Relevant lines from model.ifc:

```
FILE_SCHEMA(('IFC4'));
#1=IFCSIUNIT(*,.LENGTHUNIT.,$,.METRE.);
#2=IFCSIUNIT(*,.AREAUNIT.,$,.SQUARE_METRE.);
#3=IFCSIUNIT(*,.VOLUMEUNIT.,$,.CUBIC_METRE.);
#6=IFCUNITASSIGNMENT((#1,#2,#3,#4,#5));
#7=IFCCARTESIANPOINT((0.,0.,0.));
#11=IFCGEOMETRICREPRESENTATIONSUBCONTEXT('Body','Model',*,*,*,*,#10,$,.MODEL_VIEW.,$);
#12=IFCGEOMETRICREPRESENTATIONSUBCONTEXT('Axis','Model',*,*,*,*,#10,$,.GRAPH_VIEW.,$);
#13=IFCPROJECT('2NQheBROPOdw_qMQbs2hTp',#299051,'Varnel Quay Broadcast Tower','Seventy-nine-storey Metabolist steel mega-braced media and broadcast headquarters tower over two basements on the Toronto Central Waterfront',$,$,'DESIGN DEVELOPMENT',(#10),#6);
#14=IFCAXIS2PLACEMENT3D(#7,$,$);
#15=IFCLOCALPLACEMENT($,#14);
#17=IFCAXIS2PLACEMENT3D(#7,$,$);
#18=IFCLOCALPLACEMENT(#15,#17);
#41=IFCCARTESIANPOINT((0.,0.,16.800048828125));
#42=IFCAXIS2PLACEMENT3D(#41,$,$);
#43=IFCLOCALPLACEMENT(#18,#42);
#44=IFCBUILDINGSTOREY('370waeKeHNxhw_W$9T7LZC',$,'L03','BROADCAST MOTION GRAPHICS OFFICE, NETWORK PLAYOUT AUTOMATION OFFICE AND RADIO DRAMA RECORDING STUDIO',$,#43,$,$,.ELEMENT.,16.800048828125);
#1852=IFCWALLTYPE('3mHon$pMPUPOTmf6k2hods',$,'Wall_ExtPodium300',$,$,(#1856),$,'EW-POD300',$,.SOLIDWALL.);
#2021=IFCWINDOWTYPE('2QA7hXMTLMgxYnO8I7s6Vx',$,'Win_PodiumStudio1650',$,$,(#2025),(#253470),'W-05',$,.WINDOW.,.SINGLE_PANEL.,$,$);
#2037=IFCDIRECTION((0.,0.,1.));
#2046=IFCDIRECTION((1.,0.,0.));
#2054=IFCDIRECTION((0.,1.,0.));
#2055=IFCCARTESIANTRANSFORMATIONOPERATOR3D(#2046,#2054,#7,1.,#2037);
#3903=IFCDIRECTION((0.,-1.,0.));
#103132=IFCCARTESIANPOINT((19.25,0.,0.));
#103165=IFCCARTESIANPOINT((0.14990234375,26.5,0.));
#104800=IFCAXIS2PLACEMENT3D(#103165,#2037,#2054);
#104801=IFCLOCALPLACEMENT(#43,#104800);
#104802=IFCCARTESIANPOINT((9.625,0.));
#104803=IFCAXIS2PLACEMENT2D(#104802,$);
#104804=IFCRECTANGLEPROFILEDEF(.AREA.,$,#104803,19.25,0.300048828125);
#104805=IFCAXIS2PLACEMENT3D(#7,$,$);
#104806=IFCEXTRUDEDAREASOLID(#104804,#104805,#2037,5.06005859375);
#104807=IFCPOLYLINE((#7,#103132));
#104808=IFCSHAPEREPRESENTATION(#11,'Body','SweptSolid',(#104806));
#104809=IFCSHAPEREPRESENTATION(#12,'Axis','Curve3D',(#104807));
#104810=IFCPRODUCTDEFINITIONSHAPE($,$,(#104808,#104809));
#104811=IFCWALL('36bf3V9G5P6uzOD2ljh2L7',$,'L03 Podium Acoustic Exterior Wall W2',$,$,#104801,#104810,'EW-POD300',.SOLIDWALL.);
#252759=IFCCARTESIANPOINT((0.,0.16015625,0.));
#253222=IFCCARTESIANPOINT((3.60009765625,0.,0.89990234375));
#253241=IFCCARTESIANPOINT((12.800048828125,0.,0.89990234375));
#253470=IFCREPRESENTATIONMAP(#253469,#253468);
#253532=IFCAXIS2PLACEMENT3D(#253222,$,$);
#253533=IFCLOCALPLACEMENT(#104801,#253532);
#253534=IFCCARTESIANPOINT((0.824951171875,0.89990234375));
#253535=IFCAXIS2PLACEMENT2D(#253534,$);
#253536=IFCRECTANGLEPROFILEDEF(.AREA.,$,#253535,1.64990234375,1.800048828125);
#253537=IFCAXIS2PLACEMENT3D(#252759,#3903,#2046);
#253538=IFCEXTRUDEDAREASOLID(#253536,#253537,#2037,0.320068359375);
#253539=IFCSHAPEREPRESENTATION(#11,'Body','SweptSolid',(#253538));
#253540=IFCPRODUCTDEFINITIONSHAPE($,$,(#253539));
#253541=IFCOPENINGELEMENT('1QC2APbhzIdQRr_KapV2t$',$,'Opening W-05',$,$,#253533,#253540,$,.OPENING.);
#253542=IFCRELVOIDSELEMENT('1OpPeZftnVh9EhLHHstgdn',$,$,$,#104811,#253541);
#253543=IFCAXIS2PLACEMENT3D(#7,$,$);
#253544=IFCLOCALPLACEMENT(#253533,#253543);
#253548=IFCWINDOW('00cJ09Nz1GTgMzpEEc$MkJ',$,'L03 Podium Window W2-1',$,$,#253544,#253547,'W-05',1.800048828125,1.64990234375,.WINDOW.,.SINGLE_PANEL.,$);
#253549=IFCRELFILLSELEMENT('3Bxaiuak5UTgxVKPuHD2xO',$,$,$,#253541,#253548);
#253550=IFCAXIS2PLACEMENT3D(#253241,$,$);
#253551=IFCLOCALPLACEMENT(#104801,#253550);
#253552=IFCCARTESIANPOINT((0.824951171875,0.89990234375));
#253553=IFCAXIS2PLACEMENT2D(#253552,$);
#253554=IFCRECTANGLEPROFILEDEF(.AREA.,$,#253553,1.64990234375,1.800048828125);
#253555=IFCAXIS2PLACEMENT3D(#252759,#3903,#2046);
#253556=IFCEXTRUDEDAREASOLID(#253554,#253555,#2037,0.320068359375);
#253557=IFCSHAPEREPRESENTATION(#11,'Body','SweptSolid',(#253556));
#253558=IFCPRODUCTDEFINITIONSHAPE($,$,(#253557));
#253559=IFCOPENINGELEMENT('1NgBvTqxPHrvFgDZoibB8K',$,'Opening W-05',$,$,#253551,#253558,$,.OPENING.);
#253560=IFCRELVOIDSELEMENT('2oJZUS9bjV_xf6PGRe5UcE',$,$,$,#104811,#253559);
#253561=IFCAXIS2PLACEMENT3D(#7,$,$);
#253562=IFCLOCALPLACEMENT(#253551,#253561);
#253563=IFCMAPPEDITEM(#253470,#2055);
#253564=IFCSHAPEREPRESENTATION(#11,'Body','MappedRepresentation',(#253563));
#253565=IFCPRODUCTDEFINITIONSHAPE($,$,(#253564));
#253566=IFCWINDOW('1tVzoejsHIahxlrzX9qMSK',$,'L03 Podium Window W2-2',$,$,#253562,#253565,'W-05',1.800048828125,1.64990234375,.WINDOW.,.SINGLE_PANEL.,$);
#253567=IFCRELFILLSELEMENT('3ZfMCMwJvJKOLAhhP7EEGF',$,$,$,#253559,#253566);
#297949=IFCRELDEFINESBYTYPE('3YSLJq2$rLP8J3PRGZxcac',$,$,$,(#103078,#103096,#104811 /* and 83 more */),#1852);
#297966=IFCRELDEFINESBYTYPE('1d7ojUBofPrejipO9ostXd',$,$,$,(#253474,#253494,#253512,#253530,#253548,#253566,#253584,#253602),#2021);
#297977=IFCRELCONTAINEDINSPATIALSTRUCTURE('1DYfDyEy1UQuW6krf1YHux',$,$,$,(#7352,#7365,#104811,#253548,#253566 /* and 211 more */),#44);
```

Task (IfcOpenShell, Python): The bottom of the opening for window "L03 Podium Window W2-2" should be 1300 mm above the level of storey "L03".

```python
import numpy as np
import ifcopenshell
import ifcopenshell.api.geometry
import ifcopenshell.geom
import ifcopenshell.util.element
import ifcopenshell.util.placement
import ifcopenshell.util.shape
import ifcopenshell.util.unit

model = ifcopenshell.open("model.ifc")
unit_scale = ifcopenshell.util.unit.calculate_unit_scale(model)

window = model.by_id(253566)
opening = window.FillsVoids[0].RelatingOpeningElement
storey = ifcopenshell.util.element.get_container(window, ifc_class="IfcBuildingStorey")
level = ifcopenshell.util.placement.get_local_placement(storey.ObjectPlacement)[2, 3]

# The opening's origin need not be at the sill, so measure its lowest point.
shape = ifcopenshell.geom.create_shape(ifcopenshell.geom.settings(), opening)
bottom = ifcopenshell.util.shape.get_shape_bottom_elevation(shape, shape.geometry) / unit_scale
dz = level + 1.3 / unit_scale - bottom

shift = np.array([0.0, 0.0, dz])
# The window is placed relative to its opening, so it follows when the opening moves.
matrix = ifcopenshell.util.placement.get_local_placement(opening.ObjectPlacement)
matrix[:3, 3] += shift
ifcopenshell.api.geometry.edit_object_placement(
    model, product=opening, matrix=matrix, is_si=False, should_transform_children=True
)

print(f"moved by {dz * unit_scale:+.3f} m")

model.write("model-out.ifc")
```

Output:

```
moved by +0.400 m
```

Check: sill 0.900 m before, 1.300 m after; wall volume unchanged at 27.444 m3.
